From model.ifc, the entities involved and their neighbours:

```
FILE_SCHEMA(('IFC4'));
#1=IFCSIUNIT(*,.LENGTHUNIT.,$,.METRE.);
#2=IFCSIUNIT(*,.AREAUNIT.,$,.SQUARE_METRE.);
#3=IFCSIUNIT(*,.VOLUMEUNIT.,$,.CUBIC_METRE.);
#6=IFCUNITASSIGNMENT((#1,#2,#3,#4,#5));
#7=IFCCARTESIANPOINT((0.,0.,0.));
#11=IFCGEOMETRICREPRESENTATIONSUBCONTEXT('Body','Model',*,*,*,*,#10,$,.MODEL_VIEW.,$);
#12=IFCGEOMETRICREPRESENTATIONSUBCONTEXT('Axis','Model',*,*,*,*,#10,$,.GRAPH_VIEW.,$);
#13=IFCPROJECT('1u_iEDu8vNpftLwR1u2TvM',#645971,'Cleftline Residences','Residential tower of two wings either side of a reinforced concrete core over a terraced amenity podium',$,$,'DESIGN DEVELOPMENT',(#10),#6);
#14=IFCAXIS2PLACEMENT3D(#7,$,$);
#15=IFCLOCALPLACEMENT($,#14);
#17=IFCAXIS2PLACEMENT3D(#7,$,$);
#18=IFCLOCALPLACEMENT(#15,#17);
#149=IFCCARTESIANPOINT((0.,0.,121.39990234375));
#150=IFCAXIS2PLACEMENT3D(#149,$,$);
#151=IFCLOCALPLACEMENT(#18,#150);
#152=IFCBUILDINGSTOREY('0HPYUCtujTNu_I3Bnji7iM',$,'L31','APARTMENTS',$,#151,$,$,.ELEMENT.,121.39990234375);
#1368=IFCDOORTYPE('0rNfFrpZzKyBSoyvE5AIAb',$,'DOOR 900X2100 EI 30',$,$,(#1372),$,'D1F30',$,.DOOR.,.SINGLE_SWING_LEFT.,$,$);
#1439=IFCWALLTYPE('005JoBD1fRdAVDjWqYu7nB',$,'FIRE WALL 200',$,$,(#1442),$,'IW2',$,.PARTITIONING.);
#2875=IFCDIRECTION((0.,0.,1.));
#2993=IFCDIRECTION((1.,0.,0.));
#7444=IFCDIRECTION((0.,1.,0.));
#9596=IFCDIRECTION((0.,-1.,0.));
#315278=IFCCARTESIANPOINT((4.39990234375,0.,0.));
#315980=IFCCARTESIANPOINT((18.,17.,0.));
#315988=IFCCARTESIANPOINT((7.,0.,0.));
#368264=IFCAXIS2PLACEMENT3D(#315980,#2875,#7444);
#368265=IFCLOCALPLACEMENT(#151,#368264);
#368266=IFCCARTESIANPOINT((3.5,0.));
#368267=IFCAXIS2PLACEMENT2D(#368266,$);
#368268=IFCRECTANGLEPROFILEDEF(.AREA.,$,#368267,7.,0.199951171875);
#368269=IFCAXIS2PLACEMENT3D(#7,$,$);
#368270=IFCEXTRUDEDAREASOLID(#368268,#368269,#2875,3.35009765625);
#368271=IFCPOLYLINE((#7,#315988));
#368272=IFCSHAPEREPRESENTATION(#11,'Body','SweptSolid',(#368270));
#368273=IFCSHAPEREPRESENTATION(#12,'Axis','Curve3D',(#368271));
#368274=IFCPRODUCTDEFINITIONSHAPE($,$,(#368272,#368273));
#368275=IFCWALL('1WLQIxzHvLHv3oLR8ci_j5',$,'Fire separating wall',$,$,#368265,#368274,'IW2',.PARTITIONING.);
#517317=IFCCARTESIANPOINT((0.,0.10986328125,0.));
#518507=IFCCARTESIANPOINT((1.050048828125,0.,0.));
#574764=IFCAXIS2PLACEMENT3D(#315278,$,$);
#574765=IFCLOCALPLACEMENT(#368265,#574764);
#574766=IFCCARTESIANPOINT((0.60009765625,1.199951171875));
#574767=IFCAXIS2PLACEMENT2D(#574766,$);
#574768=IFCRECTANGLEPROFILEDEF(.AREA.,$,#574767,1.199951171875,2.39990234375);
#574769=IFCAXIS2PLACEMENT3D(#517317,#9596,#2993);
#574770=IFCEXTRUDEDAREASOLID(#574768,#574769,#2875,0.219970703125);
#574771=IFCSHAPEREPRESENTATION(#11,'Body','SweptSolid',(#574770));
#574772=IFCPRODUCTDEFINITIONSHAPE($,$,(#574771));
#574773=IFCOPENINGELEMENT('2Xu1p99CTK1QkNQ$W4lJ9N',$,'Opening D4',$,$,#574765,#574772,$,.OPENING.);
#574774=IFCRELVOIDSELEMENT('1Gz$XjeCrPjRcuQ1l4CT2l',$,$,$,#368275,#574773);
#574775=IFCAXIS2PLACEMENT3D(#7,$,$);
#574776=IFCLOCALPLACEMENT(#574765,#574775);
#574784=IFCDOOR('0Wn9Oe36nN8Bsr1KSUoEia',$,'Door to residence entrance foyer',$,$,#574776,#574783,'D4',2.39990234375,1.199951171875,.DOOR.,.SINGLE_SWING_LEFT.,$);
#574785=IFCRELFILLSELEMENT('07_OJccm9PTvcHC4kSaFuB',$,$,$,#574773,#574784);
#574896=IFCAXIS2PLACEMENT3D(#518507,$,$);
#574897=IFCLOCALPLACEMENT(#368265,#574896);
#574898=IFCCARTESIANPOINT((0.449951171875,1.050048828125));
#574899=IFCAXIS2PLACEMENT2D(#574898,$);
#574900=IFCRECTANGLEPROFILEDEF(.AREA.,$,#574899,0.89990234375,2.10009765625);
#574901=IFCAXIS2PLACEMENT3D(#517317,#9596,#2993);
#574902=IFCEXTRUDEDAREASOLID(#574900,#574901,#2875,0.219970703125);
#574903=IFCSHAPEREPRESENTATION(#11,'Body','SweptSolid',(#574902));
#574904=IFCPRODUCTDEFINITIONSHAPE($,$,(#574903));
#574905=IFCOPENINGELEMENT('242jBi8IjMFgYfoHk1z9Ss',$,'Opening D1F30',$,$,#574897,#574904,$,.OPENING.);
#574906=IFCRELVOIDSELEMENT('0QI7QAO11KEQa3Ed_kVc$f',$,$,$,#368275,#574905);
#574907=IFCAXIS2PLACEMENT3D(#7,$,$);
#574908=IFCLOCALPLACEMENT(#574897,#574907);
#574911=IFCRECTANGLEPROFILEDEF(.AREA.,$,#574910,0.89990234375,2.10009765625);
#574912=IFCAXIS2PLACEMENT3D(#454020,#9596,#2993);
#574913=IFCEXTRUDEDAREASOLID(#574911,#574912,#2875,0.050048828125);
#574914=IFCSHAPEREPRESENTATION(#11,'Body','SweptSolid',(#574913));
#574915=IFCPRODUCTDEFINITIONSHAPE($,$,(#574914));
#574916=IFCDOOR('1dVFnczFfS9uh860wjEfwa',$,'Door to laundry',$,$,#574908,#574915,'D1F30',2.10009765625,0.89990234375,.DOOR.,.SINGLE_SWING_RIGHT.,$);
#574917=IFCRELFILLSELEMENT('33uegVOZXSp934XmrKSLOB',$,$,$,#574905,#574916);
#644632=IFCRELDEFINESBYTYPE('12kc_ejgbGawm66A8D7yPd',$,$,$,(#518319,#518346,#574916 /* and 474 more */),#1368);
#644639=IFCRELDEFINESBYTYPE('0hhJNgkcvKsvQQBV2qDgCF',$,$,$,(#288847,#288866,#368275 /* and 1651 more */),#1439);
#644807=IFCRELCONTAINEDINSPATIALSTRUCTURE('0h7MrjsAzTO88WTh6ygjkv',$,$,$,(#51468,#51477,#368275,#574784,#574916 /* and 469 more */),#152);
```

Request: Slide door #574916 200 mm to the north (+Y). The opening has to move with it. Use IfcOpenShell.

```python
import ifcopenshell
import ifcopenshell.api.geometry
import ifcopenshell.util.placement
import ifcopenshell.util.unit

model = ifcopenshell.open("model.ifc")
unit_scale = ifcopenshell.util.unit.calculate_unit_scale(model)

door = model.by_guid("1dVFnczFfS9uh860wjEfwa")
opening = door.FillsVoids[0].RelatingOpeningElement
wall = opening.VoidsElements[0].RelatingBuildingElement

wall_matrix = ifcopenshell.util.placement.get_local_placement(wall.ObjectPlacement)
shift = wall_matrix[:3, 0] * 0.2 / unit_scale
before = ifcopenshell.util.placement.get_local_placement(door.ObjectPlacement)[:3, 3].copy()

# The door is placed relative to its opening, so it follows when the opening moves.
matrix = ifcopenshell.util.placement.get_local_placement(opening.ObjectPlacement)
matrix[:3, 3] += shift
ifcopenshell.api.geometry.edit_object_placement(
    model, product=opening, matrix=matrix, is_si=False, should_transform_children=True
)

after = ifcopenshell.util.placement.get_local_placement(door.ObjectPlacement)[:3, 3]
print("door moved by", (after - before).round(3) + 0.0)

model.write("model_rev.ifc")
```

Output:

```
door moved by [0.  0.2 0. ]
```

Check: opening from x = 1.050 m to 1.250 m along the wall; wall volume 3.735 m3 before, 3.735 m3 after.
